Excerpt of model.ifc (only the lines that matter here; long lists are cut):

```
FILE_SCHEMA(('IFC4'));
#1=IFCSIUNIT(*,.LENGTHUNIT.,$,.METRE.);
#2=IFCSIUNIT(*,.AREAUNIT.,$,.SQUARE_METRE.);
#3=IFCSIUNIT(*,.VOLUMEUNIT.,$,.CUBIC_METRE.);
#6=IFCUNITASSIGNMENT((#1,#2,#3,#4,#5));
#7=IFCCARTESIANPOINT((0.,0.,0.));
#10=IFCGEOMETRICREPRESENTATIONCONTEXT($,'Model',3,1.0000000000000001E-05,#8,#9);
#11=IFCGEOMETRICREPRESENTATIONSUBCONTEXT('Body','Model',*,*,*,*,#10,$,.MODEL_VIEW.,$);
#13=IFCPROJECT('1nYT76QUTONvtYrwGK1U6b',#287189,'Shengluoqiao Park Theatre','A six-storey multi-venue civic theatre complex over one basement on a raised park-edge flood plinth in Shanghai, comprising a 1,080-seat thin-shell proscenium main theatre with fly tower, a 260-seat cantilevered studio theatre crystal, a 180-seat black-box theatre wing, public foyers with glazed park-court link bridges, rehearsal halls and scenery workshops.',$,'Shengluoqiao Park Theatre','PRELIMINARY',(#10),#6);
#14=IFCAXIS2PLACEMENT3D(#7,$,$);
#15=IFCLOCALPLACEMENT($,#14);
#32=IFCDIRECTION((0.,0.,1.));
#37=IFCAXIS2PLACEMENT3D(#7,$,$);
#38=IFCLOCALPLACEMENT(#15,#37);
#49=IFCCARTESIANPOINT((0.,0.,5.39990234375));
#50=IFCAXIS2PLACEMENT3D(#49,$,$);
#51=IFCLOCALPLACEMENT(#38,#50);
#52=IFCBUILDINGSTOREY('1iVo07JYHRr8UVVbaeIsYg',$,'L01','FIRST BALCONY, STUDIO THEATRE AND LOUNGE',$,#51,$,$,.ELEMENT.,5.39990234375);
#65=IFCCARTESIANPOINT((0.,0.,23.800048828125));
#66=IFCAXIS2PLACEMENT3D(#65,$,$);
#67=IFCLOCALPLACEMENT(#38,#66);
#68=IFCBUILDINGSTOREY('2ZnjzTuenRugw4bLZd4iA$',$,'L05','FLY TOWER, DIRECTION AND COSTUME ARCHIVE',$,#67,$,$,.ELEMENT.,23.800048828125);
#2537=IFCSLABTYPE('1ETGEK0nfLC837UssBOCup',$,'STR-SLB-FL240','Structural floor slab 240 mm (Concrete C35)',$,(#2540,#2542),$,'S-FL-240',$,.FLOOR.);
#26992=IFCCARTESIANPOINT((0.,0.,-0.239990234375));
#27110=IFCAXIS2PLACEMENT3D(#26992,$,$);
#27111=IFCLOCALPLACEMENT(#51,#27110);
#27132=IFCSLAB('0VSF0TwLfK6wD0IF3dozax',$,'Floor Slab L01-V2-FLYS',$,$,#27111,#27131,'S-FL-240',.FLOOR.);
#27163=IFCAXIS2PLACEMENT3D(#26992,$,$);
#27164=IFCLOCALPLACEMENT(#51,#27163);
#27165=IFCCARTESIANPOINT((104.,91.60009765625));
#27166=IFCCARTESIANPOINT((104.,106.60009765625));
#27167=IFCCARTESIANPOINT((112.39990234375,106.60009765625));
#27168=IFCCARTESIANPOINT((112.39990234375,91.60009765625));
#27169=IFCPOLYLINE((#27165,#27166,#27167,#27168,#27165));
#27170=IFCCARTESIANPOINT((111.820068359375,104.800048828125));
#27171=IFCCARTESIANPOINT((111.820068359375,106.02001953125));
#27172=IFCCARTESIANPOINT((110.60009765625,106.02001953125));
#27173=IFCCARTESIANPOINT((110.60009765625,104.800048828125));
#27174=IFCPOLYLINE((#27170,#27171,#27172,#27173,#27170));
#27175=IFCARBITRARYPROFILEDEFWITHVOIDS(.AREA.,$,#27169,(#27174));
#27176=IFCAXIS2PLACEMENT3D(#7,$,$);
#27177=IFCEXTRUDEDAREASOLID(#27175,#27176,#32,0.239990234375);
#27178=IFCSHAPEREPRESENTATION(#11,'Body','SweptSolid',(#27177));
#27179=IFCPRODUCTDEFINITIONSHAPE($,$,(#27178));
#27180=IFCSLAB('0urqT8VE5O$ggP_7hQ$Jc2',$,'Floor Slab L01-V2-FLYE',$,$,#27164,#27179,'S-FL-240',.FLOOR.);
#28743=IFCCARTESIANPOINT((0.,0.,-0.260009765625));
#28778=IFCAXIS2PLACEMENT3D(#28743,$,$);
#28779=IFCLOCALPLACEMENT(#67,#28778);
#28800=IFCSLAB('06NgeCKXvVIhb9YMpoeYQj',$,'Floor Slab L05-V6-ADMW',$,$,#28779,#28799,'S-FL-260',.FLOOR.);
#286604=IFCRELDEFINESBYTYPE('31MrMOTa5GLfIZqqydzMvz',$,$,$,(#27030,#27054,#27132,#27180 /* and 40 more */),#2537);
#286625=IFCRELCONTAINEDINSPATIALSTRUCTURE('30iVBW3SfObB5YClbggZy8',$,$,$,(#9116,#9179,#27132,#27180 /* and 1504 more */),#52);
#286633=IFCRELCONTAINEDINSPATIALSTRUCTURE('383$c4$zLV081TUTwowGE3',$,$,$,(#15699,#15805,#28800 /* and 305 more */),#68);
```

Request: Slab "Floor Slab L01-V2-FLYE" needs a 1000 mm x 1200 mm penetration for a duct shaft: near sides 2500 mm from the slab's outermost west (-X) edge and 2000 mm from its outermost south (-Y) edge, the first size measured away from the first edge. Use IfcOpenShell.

```python
import numpy as np
import ifcopenshell
import ifcopenshell.api.feature
import ifcopenshell.api.geometry
import ifcopenshell.api.root
import ifcopenshell.geom
import ifcopenshell.util.placement
import ifcopenshell.util.representation
import ifcopenshell.util.shape
import ifcopenshell.util.unit

model = ifcopenshell.open("model.ifc")
unit_scale = ifcopenshell.util.unit.calculate_unit_scale(model)
settings = ifcopenshell.geom.settings()


def volume(element):
    """Net volume in cubic metres, openings subtracted."""
    shape = ifcopenshell.geom.create_shape(settings, element)
    return ifcopenshell.util.shape.get_volume(shape.geometry)


slab = model.by_guid("0urqT8VE5O$ggP_7hQ$Jc2")
before = volume(slab)

# Extent in the slab's own axes, in metres. The edges named are its -X and -Y sides.
slab_shape = ifcopenshell.geom.create_shape(settings, slab)
vertices = ifcopenshell.util.shape.get_vertices(slab_shape.geometry)
x_min, y_min, bottom = vertices.min(axis=0)
top = vertices[:, 2].max()

opening = ifcopenshell.api.root.create_entity(model, ifc_class="IfcOpeningElement", name="Duct shaft opening", predefined_type="OPENING")
context = ifcopenshell.util.representation.get_context(model, "Model", "Body", "MODEL_VIEW")
width, depth = 1, 1.2
outline = [(0.0, 0.0), (width, 0.0), (width, depth), (0.0, depth), (0.0, 0.0)]
# Overshoot both faces by 50 mm so the cut is clean.
shape = ifcopenshell.api.geometry.add_slab_representation(
    model, context=context, depth=top - bottom + 0.1, polyline=outline
)
ifcopenshell.api.geometry.assign_representation(model, product=opening, representation=shape)

matrix = ifcopenshell.util.placement.get_local_placement(slab.ObjectPlacement)
matrix[:, 3] = matrix @ np.append(np.array([x_min + 2.5, y_min + 2, bottom - 0.05]) / unit_scale, 1.0)
ifcopenshell.api.geometry.edit_object_placement(model, product=opening, matrix=matrix, is_si=False)
ifcopenshell.api.feature.add_feature(model, feature=opening, element=slab)

after = volume(slab)

print(f"slab volume {before:.3f} -> {after:.3f} m3")

model.write("model_edited.ifc")
```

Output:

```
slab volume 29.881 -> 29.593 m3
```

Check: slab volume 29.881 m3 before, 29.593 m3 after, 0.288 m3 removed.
